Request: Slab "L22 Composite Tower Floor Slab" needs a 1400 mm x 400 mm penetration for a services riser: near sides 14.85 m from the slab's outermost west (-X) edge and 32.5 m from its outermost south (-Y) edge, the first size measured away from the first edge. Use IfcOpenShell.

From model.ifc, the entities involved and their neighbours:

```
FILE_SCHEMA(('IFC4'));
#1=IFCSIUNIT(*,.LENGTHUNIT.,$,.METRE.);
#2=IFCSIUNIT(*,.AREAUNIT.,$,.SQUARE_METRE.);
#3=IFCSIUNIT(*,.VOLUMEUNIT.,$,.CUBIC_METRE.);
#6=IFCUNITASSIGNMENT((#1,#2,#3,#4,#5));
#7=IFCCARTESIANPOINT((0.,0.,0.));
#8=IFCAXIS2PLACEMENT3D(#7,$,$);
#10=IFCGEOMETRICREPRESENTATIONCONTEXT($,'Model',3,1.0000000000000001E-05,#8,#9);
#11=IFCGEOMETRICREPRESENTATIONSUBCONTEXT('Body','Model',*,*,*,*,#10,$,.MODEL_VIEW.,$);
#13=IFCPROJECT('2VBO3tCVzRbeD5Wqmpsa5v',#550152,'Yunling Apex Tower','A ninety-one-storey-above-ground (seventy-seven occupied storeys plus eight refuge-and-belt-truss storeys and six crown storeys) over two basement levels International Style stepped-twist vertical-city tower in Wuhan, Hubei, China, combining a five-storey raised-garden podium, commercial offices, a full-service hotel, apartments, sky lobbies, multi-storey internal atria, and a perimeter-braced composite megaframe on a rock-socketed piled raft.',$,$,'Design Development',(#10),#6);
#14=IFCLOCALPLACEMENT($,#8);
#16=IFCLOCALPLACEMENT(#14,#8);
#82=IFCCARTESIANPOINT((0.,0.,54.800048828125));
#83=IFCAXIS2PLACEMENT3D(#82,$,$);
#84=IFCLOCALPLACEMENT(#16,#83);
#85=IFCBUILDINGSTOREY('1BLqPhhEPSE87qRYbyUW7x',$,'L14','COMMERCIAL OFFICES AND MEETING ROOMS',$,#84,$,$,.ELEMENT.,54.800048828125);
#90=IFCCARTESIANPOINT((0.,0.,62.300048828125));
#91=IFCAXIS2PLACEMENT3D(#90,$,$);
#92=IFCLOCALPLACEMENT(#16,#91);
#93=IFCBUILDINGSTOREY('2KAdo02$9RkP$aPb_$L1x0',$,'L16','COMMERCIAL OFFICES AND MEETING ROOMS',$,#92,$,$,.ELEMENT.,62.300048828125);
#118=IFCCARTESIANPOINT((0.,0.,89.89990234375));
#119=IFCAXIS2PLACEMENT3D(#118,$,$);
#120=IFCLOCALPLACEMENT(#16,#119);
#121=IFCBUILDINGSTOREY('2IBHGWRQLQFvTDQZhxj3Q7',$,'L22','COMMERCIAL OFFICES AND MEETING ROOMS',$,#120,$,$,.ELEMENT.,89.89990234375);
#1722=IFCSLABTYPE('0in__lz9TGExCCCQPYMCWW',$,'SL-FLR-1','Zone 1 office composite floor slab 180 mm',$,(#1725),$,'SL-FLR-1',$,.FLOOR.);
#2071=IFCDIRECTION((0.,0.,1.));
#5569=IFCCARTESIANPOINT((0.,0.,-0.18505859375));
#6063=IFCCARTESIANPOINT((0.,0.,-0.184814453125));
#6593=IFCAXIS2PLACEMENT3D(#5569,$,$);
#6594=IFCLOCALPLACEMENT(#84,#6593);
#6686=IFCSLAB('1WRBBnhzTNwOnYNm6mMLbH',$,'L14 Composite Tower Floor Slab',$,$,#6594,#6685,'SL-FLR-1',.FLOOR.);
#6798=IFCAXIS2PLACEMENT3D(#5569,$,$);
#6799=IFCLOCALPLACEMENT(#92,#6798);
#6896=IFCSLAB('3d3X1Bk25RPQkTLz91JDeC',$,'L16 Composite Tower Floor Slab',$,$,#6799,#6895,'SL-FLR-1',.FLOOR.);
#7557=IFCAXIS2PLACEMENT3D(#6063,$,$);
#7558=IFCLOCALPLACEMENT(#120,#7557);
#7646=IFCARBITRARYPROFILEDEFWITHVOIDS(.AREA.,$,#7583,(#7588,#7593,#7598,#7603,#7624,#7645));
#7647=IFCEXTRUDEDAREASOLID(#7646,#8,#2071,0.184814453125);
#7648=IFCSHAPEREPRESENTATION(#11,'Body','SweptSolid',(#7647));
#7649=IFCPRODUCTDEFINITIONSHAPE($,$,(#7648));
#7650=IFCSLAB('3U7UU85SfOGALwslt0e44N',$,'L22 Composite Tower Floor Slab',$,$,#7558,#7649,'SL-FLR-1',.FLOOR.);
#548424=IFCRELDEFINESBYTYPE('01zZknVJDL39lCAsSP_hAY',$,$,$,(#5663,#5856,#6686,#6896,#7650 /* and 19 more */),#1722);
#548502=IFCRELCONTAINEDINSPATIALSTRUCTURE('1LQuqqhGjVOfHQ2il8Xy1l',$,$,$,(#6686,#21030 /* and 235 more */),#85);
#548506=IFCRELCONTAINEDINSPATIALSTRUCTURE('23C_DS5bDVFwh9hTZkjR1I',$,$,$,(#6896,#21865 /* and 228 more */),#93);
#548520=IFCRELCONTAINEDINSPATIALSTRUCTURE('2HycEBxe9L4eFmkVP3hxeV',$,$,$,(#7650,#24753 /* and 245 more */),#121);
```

```python
import numpy as np
import ifcopenshell
import ifcopenshell.api.feature
import ifcopenshell.api.geometry
import ifcopenshell.api.root
import ifcopenshell.geom
import ifcopenshell.util.placement
import ifcopenshell.util.representation
import ifcopenshell.util.shape
import ifcopenshell.util.unit

model = ifcopenshell.open("model.ifc")
unit_scale = ifcopenshell.util.unit.calculate_unit_scale(model)
settings = ifcopenshell.geom.settings()


def volume(element):
    """Net volume in cubic metres, openings subtracted."""
    shape = ifcopenshell.geom.create_shape(settings, element)
    return ifcopenshell.util.shape.get_volume(shape.geometry)


slab = model.by_guid("3U7UU85SfOGALwslt0e44N")
before = volume(slab)

# Extent in the slab's own axes, in metres. The edges named are its -X and -Y sides.
slab_shape = ifcopenshell.geom.create_shape(settings, slab)
vertices = ifcopenshell.util.shape.get_vertices(slab_shape.geometry)
x_min, y_min, bottom = vertices.min(axis=0)
top = vertices[:, 2].max()

opening = ifcopenshell.api.root.create_entity(model, ifc_class="IfcOpeningElement", name="Services riser opening", predefined_type="OPENING")
context = ifcopenshell.util.representation.get_context(model, "Model", "Body", "MODEL_VIEW")
width, depth = 1.4, 0.4
outline = [(0.0, 0.0), (width, 0.0), (width, depth), (0.0, depth), (0.0, 0.0)]
# Overshoot both faces by 50 mm so the cut is clean.
shape = ifcopenshell.api.geometry.add_slab_representation(
    model, context=context, depth=top - bottom + 0.1, polyline=outline
)
ifcopenshell.api.geometry.assign_representation(model, product=opening, representation=shape)

matrix = ifcopenshell.util.placement.get_local_placement(slab.ObjectPlacement)
matrix[:, 3] = matrix @ np.append(np.array([x_min + 14.85, y_min + 32.5, bottom - 0.05]) / unit_scale, 1.0)
ifcopenshell.api.geometry.edit_object_placement(model, product=opening, matrix=matrix, is_si=False)
ifcopenshell.api.feature.add_feature(model, feature=opening, element=slab)

after = volume(slab)

print(f"slab volume {before:.3f} -> {after:.3f} m3")

model.write("model_updated.ifc")
```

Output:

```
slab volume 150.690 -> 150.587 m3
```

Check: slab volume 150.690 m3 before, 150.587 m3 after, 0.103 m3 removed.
